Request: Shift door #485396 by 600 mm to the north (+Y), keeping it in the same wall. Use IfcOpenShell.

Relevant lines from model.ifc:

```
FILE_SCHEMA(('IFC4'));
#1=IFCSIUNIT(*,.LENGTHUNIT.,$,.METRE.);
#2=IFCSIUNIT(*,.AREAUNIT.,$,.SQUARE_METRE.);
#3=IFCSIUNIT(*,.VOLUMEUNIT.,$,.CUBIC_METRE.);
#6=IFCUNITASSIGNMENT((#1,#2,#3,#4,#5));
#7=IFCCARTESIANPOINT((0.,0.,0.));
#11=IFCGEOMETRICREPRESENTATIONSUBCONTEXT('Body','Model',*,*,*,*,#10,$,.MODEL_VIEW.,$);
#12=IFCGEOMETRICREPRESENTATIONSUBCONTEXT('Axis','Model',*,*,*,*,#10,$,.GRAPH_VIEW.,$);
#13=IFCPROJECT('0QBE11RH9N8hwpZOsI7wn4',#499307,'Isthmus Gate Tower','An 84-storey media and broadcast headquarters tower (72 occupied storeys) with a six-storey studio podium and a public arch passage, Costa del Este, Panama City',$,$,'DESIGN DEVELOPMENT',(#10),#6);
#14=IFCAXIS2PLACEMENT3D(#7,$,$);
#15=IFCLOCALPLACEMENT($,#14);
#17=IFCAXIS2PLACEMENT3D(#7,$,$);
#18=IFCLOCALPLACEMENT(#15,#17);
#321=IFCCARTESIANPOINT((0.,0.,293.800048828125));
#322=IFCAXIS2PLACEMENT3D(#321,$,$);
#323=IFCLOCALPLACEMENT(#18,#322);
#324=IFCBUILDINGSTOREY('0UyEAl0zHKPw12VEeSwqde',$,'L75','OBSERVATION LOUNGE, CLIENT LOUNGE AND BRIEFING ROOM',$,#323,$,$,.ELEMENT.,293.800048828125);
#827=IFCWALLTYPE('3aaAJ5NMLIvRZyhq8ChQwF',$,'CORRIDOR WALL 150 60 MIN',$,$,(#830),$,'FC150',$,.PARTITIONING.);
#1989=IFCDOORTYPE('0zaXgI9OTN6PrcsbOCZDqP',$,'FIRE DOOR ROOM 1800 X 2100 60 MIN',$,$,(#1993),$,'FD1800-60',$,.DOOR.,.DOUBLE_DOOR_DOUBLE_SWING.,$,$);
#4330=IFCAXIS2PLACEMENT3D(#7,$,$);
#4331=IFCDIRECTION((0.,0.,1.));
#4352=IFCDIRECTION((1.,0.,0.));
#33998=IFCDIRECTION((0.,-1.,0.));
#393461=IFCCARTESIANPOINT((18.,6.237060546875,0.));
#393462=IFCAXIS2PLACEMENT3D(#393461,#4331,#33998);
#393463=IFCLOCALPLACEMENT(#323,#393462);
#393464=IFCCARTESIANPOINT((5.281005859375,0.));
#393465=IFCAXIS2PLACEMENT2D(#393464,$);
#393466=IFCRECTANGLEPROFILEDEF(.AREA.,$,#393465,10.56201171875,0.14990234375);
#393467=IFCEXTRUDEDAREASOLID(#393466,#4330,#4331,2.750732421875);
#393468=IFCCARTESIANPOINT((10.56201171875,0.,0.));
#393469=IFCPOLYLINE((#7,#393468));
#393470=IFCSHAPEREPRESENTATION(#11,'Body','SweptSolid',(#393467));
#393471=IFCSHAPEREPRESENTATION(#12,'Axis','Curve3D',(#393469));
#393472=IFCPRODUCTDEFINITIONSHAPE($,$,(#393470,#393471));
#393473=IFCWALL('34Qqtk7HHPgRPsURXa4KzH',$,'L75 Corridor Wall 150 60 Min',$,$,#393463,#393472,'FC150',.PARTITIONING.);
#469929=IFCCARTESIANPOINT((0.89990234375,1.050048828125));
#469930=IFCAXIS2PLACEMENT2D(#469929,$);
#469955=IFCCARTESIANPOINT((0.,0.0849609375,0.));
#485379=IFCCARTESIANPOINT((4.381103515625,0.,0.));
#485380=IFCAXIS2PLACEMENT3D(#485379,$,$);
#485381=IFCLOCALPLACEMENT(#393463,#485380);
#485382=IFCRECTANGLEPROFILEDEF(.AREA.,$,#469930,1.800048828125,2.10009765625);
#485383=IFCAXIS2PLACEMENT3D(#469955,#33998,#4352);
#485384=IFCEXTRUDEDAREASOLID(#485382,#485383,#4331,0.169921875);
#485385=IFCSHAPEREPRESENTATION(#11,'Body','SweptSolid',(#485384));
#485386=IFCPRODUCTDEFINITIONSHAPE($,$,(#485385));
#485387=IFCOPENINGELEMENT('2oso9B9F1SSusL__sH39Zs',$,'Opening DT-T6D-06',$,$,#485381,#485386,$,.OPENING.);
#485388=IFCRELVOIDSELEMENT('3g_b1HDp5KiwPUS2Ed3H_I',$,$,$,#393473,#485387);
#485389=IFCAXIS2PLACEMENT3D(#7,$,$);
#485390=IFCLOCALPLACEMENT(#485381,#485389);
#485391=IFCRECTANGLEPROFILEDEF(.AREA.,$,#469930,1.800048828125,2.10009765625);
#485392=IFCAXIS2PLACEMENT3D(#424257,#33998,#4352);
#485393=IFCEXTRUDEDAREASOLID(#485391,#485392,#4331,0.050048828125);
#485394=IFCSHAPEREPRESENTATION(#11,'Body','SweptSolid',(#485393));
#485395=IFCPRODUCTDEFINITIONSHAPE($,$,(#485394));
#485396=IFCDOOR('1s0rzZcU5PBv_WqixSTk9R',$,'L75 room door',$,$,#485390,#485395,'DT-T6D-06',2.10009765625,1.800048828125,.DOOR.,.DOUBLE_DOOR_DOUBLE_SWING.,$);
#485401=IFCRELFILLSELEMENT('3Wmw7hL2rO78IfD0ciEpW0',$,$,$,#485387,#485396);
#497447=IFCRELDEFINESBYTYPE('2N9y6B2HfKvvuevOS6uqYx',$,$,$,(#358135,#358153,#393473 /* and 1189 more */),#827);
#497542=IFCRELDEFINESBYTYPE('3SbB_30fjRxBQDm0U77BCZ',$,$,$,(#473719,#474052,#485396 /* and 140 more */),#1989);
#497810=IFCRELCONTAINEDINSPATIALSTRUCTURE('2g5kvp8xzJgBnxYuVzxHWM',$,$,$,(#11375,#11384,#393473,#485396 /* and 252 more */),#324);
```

```python
import ifcopenshell
import ifcopenshell.api.geometry
import ifcopenshell.util.placement

model = ifcopenshell.open("model.ifc")

door = model.by_guid("1s0rzZcU5PBv_WqixSTk9R")
opening = door.FillsVoids[0].RelatingOpeningElement
wall = opening.VoidsElements[0].RelatingBuildingElement

wall_matrix = ifcopenshell.util.placement.get_local_placement(wall.ObjectPlacement)
shift = wall_matrix[:3, 0] * -0.6
before = ifcopenshell.util.placement.get_local_placement(door.ObjectPlacement)[:3, 3].copy()

# The door is placed relative to its opening, so it follows when the opening moves.
matrix = ifcopenshell.util.placement.get_local_placement(opening.ObjectPlacement)
matrix[:3, 3] += shift
ifcopenshell.api.geometry.edit_object_placement(
    model, product=opening, matrix=matrix, is_si=False, should_transform_children=True
)

after = ifcopenshell.util.placement.get_local_placement(door.ObjectPlacement)[:3, 3]
print("door moved by", (after - before).round(3) + 0.0)

model.write("model_v2.ifc")
```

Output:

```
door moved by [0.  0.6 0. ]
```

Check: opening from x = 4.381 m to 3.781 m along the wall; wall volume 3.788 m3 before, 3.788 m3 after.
